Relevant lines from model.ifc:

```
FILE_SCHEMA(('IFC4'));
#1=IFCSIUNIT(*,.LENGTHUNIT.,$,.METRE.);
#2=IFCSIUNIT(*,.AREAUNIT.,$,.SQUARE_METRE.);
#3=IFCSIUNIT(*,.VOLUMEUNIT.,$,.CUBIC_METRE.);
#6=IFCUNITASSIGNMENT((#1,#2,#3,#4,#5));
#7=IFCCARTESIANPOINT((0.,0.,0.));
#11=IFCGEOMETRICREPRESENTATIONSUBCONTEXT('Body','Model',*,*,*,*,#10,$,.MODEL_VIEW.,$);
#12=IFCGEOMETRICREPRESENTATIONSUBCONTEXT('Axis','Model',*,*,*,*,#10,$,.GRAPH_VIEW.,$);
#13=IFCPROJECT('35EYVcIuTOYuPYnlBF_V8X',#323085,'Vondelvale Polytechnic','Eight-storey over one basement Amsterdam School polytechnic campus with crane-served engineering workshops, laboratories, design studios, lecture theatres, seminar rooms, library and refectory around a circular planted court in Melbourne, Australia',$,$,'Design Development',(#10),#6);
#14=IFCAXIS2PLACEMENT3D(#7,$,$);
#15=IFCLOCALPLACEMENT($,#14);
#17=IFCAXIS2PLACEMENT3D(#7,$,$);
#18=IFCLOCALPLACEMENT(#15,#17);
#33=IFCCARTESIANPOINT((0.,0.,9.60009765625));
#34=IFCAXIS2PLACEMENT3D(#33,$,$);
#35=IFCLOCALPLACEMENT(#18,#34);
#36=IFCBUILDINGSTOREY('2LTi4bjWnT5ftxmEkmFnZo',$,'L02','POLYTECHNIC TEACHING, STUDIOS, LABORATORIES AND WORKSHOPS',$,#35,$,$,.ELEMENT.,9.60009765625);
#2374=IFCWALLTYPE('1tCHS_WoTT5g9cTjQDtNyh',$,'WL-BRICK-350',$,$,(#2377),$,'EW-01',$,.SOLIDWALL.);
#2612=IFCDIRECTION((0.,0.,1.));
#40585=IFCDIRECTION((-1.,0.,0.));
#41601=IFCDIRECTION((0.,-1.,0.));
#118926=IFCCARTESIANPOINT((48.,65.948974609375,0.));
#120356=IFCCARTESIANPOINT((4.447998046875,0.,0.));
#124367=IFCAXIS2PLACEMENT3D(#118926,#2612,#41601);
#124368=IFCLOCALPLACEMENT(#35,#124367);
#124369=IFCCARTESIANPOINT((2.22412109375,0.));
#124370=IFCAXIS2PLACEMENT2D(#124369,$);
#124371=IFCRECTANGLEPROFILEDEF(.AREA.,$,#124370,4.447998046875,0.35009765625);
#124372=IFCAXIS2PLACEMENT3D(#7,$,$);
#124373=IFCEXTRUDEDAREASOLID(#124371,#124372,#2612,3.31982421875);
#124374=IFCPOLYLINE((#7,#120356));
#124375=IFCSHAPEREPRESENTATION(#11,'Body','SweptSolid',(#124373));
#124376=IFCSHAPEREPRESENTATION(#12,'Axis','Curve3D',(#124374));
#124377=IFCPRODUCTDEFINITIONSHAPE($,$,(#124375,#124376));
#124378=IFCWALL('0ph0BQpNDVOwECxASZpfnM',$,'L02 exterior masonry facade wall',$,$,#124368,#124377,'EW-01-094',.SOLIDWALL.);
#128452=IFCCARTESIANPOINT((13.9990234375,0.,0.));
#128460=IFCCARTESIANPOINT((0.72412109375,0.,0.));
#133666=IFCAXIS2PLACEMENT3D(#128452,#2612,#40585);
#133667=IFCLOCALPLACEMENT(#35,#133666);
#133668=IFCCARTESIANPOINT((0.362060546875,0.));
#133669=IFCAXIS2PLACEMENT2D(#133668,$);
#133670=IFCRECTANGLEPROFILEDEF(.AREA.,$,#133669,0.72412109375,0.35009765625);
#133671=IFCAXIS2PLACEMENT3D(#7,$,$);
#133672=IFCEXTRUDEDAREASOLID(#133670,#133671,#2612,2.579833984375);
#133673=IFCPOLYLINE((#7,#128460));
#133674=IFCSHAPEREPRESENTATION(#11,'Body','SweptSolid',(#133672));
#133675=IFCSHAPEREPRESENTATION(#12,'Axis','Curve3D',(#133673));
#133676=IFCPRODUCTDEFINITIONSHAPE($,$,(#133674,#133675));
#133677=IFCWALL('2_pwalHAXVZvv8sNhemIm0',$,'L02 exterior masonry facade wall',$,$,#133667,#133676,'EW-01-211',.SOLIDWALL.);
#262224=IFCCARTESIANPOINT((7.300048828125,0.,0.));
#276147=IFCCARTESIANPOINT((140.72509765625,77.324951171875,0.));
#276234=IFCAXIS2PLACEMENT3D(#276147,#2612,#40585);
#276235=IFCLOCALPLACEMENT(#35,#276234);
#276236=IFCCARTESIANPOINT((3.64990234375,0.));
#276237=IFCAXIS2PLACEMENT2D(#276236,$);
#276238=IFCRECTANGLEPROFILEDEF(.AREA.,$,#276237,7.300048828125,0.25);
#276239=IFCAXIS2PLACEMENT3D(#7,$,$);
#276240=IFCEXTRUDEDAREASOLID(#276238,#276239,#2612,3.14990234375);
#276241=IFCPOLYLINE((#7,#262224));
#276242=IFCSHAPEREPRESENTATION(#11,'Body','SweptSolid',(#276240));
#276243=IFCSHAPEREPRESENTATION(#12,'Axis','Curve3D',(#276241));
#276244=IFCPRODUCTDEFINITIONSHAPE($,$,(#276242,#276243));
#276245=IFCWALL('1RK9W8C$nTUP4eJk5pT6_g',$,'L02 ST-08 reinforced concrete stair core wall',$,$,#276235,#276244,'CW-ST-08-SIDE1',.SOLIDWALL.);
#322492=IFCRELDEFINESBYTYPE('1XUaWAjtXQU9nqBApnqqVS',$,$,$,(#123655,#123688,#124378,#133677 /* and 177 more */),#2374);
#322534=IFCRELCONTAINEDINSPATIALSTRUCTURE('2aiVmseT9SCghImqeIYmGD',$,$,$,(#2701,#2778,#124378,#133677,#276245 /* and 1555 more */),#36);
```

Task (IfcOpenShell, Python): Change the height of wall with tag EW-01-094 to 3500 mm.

```python
import ifcopenshell
import ifcopenshell.geom
import ifcopenshell.util.representation
import ifcopenshell.util.shape
import ifcopenshell.util.unit

model = ifcopenshell.open("model.ifc")
unit_scale = ifcopenshell.util.unit.calculate_unit_scale(model)
settings = ifcopenshell.geom.settings()


def volume(element):
    """Net volume in cubic metres, openings subtracted."""
    shape = ifcopenshell.geom.create_shape(settings, element)
    return ifcopenshell.util.shape.get_volume(shape.geometry)


wall = model.by_guid("0ph0BQpNDVOwECxASZpfnM")
before = volume(wall)

body = ifcopenshell.util.representation.get_representation(wall, "Model", "Body")
solid = body.Items[0]
old_height = solid.Depth
solid.Depth = 3.5 / unit_scale
after = volume(wall)

print(f"height {old_height:g} -> {solid.Depth:g}, volume {before:.3f} -> {after:.3f} m3")

model.write("model_v2.ifc")
```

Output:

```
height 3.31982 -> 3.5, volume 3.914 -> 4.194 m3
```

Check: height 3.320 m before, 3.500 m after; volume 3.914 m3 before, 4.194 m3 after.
